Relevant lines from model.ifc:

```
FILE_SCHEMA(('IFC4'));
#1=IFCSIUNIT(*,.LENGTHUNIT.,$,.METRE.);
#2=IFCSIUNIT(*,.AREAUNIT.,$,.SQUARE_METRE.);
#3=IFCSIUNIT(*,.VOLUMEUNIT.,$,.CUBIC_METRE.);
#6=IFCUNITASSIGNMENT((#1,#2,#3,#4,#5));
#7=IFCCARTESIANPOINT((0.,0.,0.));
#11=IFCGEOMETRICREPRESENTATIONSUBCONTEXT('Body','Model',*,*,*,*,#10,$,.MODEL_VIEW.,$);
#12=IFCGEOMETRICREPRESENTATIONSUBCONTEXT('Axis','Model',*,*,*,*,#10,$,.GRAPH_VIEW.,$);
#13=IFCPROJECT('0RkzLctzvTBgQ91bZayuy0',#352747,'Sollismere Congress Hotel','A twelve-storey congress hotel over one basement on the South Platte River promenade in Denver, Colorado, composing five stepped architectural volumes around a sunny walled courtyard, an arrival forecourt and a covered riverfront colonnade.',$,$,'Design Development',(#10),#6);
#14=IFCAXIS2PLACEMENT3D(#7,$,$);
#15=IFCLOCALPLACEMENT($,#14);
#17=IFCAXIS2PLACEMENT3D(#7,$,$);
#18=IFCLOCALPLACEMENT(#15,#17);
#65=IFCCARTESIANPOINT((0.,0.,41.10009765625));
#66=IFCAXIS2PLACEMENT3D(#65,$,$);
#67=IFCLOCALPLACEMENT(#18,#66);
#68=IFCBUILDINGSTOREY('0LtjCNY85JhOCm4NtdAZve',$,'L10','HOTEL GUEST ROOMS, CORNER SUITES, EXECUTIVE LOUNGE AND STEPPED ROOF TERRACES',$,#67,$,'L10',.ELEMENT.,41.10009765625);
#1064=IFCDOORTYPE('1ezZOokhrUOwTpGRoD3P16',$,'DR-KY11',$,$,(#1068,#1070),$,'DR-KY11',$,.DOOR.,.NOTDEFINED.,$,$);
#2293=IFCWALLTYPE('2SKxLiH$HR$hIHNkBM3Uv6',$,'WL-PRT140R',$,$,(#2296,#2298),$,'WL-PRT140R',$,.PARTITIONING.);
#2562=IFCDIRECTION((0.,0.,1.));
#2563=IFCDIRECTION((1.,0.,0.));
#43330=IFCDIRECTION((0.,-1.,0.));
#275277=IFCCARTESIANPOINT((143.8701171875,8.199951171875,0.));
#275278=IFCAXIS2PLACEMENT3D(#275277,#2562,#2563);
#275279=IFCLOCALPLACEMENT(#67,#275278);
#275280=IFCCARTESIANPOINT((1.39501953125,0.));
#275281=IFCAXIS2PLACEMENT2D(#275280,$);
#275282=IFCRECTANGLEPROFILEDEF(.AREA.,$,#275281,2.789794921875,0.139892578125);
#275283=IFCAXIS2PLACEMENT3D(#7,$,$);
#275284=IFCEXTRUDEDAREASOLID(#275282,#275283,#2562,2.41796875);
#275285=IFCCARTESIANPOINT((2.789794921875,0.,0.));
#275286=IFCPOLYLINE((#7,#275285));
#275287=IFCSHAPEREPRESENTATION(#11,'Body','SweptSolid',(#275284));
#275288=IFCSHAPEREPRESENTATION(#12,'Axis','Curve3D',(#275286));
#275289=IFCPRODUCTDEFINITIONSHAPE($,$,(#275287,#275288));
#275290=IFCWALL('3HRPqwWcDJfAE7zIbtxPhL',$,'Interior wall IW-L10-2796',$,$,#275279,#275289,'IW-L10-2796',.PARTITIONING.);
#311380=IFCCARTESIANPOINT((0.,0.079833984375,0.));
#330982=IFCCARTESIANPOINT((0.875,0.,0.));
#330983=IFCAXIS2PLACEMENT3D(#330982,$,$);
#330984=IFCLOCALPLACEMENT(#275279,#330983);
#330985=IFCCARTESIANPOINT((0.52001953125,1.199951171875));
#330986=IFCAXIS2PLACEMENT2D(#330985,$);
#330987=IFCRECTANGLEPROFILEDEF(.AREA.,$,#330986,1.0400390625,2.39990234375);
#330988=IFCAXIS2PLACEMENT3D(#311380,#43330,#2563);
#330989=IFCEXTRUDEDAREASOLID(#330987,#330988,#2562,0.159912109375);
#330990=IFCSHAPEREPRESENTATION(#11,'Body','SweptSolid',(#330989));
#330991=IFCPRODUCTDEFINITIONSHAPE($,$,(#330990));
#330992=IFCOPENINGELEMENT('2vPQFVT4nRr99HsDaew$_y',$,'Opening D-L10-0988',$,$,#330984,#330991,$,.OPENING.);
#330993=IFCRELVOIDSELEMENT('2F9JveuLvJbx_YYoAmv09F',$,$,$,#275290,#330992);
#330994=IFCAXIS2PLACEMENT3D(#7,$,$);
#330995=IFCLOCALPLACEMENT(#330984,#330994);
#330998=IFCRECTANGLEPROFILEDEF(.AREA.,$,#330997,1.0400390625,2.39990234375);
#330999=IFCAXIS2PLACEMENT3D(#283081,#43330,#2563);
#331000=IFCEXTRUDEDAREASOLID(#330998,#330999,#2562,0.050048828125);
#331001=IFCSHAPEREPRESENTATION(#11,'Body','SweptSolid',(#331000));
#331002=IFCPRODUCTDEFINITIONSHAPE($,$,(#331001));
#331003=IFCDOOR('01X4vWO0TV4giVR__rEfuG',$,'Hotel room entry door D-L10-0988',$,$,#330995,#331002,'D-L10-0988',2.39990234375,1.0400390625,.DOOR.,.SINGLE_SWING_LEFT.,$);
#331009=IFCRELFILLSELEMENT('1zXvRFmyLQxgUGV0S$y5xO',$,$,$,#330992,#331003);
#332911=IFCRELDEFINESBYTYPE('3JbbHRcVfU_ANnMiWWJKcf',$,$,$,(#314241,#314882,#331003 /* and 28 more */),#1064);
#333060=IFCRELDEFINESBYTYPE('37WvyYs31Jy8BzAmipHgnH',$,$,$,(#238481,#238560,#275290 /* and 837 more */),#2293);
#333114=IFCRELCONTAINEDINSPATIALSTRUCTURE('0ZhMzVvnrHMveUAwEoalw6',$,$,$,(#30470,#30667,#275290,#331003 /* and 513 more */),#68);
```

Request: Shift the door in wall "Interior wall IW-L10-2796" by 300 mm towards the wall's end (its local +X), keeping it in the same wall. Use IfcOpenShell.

```python
import ifcopenshell
import ifcopenshell.api.geometry
import ifcopenshell.util.placement
import ifcopenshell.util.unit

model = ifcopenshell.open("model.ifc")
unit_scale = ifcopenshell.util.unit.calculate_unit_scale(model)

door = model.by_id(331003)
opening = door.FillsVoids[0].RelatingOpeningElement
wall = opening.VoidsElements[0].RelatingBuildingElement

wall_matrix = ifcopenshell.util.placement.get_local_placement(wall.ObjectPlacement)
shift = wall_matrix[:3, 0] * 0.3 / unit_scale
before = ifcopenshell.util.placement.get_local_placement(door.ObjectPlacement)[:3, 3].copy()

# The door is placed relative to its opening, so it follows when the opening moves.
matrix = ifcopenshell.util.placement.get_local_placement(opening.ObjectPlacement)
matrix[:3, 3] += shift
ifcopenshell.api.geometry.edit_object_placement(
    model, product=opening, matrix=matrix, is_si=False, should_transform_children=True
)

after = ifcopenshell.util.placement.get_local_placement(door.ObjectPlacement)[:3, 3]
print("door moved by", (after - before).round(3) + 0.0)

model.write("model_rev.ifc")
```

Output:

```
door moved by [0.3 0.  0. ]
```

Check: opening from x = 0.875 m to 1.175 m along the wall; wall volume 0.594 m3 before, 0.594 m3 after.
